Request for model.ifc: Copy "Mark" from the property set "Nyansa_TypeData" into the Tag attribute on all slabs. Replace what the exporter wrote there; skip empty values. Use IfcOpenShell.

First a look at what the model holds.

```python
import ifcopenshell
import ifcopenshell.util.element

model = ifcopenshell.open("model.ifc")
print(model.schema)
slabs = model.by_type("IfcSlab")
print(len(slabs), "slabs")
for e in slabs[:8]:
    source = ifcopenshell.util.element.get_pset(e, "Nyansa_TypeData", "Mark")
    target = e.Tag
    print(e.id(), repr(source), repr(target), sep=" | ")
```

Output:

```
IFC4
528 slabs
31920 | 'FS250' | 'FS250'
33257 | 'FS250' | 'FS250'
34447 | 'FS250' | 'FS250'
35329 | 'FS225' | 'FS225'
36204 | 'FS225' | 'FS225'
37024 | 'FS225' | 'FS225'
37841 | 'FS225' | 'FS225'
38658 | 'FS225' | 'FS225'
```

```python
import ifcopenshell
import ifcopenshell.util.element

model = ifcopenshell.open("model.ifc")

count = 0
for e in model.by_type("IfcSlab"):
    value = ifcopenshell.util.element.get_pset(e, "Nyansa_TypeData", "Mark")
    current = e.Tag
    if not value or not value.strip() or current == value:
        continue
    e.Tag = value
    count += 1

print(count, "slabs updated")

model.write("model_rev.ifc")
```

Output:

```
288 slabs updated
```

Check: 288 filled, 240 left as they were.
